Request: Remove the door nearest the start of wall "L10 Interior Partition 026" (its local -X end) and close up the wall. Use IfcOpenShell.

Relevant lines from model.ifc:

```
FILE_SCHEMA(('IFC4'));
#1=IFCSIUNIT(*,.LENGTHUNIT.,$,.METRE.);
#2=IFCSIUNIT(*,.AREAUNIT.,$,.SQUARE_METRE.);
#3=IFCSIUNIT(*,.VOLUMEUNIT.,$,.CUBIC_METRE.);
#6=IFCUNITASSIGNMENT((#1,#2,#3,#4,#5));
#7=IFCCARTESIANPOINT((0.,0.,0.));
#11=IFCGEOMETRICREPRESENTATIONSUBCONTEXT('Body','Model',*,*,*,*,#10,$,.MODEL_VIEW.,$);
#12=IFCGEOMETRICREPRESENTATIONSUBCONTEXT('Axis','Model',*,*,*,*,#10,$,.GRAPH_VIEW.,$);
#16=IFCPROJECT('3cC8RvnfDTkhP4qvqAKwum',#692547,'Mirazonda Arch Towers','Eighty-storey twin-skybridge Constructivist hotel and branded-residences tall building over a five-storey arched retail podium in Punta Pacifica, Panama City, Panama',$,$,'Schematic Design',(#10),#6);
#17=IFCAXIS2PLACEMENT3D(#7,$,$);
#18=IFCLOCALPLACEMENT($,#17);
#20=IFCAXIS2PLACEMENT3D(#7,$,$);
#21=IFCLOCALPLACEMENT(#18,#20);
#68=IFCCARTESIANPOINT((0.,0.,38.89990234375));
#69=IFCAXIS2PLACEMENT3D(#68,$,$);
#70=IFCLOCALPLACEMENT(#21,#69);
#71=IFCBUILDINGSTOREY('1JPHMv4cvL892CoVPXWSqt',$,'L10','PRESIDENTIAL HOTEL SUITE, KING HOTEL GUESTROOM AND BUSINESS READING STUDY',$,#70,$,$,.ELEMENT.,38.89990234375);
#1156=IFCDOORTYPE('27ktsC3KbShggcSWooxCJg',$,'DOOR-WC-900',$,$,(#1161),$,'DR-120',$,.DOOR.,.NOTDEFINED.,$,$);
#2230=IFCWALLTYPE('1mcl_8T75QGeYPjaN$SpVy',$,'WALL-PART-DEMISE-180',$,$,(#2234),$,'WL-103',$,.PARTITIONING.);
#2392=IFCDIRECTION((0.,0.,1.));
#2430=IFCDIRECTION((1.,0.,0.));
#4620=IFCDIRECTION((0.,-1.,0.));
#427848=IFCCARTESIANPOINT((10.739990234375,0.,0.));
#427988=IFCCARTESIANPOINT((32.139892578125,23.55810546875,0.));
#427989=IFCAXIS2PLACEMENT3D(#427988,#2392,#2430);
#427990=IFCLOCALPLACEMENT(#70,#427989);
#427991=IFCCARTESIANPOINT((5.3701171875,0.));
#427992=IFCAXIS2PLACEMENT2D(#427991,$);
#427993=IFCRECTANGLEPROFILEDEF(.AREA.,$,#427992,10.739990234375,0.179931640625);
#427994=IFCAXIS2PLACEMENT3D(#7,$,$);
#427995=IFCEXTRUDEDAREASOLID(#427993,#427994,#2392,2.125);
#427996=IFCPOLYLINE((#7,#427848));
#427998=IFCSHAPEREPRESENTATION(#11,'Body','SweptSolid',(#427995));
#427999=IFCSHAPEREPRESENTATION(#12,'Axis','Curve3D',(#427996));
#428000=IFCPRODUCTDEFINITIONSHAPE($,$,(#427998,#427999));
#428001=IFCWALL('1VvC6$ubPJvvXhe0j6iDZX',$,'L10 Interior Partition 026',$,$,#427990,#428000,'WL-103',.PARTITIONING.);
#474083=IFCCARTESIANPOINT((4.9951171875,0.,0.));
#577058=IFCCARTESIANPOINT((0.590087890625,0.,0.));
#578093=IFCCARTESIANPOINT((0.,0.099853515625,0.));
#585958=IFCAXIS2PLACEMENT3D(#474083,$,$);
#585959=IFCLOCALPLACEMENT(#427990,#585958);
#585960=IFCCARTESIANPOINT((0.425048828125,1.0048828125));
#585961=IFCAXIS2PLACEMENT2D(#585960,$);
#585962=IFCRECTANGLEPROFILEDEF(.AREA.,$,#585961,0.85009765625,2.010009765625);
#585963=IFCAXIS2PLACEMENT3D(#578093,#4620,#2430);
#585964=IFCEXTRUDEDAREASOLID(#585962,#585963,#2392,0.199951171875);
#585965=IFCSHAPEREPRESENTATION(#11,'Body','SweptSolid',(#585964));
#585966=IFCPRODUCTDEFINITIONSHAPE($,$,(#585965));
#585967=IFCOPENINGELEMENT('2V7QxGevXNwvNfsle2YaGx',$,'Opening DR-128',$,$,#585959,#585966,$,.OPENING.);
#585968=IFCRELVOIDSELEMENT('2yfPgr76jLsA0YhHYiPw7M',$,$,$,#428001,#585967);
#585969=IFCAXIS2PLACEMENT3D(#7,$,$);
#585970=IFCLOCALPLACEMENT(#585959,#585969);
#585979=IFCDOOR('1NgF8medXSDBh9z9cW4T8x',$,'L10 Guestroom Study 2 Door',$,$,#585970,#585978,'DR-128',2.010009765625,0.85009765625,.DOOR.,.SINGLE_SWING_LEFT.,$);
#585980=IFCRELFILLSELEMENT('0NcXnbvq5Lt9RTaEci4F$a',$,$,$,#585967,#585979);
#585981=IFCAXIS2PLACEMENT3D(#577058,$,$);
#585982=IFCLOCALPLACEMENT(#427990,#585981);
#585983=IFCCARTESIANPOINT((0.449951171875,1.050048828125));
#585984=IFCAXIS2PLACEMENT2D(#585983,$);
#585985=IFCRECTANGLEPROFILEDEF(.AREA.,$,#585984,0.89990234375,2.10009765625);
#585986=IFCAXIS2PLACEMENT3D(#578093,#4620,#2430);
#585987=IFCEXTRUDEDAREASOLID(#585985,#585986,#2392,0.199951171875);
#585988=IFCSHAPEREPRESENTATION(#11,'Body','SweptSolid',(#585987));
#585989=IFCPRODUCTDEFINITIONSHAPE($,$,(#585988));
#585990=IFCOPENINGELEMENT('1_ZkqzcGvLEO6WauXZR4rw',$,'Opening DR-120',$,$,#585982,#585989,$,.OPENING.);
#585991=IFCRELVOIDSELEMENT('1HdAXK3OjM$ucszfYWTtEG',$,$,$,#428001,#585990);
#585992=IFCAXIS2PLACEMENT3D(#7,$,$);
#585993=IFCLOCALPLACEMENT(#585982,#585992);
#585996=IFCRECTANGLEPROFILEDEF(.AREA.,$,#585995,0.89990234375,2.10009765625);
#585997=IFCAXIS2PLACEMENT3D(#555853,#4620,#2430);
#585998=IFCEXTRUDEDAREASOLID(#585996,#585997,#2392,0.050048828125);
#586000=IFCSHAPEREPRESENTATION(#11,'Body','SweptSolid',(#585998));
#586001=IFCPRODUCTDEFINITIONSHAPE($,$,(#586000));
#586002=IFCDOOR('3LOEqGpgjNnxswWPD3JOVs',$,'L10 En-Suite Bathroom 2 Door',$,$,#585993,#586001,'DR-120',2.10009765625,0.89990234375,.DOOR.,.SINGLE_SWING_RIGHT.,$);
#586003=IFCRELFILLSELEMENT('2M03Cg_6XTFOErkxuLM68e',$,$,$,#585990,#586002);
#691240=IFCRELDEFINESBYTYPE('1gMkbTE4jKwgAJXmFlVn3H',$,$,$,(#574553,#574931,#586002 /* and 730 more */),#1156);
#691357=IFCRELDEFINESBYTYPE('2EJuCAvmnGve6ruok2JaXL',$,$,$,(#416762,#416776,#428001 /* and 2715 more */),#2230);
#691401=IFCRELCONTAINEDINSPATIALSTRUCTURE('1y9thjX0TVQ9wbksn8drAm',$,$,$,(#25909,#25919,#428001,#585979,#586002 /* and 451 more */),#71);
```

```python
import ifcopenshell
import ifcopenshell.api.feature
import ifcopenshell.api.root
import ifcopenshell.geom
import ifcopenshell.util.shape

model = ifcopenshell.open("model.ifc")
settings = ifcopenshell.geom.settings()


def volume(element):
    """Net volume in cubic metres, openings subtracted."""
    shape = ifcopenshell.geom.create_shape(settings, element)
    return ifcopenshell.util.shape.get_volume(shape.geometry)


door = model.by_guid("3LOEqGpgjNnxswWPD3JOVs")
opening = door.FillsVoids[0].RelatingOpeningElement
wall = opening.VoidsElements[0].RelatingBuildingElement
before = volume(wall)

ifcopenshell.api.root.remove_product(model, product=door)
ifcopenshell.api.feature.remove_feature(model, feature=opening)

after = volume(wall)

print(f"wall volume {before:.3f} -> {after:.3f} m3")

model.write("model_edited.ifc")
```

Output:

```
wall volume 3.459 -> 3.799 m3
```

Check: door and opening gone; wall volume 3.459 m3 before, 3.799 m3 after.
